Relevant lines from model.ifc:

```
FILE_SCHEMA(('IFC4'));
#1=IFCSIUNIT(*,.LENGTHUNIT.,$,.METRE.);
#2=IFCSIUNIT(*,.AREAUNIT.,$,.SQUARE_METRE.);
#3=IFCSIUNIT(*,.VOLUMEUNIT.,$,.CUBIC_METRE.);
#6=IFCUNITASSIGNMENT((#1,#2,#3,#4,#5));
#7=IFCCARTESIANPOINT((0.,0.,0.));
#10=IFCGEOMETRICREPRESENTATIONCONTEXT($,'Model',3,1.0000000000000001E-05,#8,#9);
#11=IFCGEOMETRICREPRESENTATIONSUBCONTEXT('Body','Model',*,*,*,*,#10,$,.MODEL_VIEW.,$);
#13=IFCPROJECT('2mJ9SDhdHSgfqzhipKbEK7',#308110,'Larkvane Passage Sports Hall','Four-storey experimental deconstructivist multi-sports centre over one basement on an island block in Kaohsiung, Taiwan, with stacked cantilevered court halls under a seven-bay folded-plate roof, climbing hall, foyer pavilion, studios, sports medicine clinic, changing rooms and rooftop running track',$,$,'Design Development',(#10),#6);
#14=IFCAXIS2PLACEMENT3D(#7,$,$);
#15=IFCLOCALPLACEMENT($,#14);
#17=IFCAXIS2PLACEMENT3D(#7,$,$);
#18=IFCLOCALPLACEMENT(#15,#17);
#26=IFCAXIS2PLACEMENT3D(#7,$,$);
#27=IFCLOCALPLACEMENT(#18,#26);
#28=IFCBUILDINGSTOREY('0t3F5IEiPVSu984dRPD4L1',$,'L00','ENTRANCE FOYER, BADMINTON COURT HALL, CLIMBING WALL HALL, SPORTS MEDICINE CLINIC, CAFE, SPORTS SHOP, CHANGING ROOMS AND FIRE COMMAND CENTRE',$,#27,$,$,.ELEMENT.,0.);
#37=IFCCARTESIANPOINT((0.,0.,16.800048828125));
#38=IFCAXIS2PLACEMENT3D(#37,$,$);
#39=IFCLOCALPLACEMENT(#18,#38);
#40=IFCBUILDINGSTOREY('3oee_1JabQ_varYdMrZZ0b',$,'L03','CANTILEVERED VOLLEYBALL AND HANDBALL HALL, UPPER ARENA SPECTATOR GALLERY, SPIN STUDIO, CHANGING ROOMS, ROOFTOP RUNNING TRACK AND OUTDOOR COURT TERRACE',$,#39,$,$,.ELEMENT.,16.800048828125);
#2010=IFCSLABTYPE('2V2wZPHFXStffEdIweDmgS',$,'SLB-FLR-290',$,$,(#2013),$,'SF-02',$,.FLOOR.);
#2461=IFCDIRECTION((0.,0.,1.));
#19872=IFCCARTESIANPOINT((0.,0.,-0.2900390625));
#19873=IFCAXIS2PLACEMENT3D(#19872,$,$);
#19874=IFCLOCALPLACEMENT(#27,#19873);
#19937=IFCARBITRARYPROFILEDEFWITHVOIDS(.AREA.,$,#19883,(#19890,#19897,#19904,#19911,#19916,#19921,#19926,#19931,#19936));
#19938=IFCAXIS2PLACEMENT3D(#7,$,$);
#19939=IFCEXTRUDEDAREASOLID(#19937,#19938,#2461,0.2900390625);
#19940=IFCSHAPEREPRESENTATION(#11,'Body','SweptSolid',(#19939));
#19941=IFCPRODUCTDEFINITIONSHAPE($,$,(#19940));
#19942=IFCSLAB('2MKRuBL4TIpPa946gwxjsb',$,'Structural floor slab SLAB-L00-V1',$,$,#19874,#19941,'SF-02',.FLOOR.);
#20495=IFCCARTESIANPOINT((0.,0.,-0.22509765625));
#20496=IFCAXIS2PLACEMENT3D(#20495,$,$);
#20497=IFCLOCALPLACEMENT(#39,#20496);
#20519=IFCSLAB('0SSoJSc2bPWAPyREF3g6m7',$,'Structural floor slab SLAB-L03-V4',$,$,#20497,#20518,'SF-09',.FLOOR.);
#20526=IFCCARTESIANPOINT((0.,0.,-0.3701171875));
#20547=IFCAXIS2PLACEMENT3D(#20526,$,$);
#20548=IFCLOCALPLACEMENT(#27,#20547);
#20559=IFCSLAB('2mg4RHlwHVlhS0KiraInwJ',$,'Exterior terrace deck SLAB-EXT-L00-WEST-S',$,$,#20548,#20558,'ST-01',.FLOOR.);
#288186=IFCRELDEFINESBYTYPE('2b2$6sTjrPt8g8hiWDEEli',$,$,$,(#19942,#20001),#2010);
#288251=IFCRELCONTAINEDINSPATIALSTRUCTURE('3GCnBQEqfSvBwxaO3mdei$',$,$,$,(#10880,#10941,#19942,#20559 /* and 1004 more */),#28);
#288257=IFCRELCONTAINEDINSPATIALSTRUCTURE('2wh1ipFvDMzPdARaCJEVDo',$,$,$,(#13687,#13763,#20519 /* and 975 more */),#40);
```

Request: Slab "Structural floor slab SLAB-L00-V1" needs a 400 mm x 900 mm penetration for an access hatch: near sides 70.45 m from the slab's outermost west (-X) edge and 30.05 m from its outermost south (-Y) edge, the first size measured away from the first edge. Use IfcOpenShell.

```python
import numpy as np
import ifcopenshell
import ifcopenshell.api.feature
import ifcopenshell.api.geometry
import ifcopenshell.api.root
import ifcopenshell.geom
import ifcopenshell.util.placement
import ifcopenshell.util.representation
import ifcopenshell.util.shape
import ifcopenshell.util.unit

model = ifcopenshell.open("model.ifc")
unit_scale = ifcopenshell.util.unit.calculate_unit_scale(model)
settings = ifcopenshell.geom.settings()


def volume(element):
    """Net volume in cubic metres, openings subtracted."""
    shape = ifcopenshell.geom.create_shape(settings, element)
    return ifcopenshell.util.shape.get_volume(shape.geometry)


slab = model.by_guid("2MKRuBL4TIpPa946gwxjsb")
before = volume(slab)

# Extent in the slab's own axes, in metres. The edges named are its -X and -Y sides.
slab_shape = ifcopenshell.geom.create_shape(settings, slab)
vertices = ifcopenshell.util.shape.get_vertices(slab_shape.geometry)
x_min, y_min, bottom = vertices.min(axis=0)
top = vertices[:, 2].max()

opening = ifcopenshell.api.root.create_entity(model, ifc_class="IfcOpeningElement", name="Access hatch opening", predefined_type="OPENING")
context = ifcopenshell.util.representation.get_context(model, "Model", "Body", "MODEL_VIEW")
width, depth = 0.4, 0.9
outline = [(0.0, 0.0), (width, 0.0), (width, depth), (0.0, depth), (0.0, 0.0)]
# Overshoot both faces by 50 mm so the cut is clean.
shape = ifcopenshell.api.geometry.add_slab_representation(
    model, context=context, depth=top - bottom + 0.1, polyline=outline
)
ifcopenshell.api.geometry.assign_representation(model, product=opening, representation=shape)

matrix = ifcopenshell.util.placement.get_local_placement(slab.ObjectPlacement)
matrix[:, 3] = matrix @ np.append(np.array([x_min + 70.45, y_min + 30.05, bottom - 0.05]) / unit_scale, 1.0)
ifcopenshell.api.geometry.edit_object_placement(model, product=opening, matrix=matrix, is_si=False)
ifcopenshell.api.feature.add_feature(model, feature=opening, element=slab)

after = volume(slab)

print(f"slab volume {before:.3f} -> {after:.3f} m3")

model.write("model_edited.ifc")
```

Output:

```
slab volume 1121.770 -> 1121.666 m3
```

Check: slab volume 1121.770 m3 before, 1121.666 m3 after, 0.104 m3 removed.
